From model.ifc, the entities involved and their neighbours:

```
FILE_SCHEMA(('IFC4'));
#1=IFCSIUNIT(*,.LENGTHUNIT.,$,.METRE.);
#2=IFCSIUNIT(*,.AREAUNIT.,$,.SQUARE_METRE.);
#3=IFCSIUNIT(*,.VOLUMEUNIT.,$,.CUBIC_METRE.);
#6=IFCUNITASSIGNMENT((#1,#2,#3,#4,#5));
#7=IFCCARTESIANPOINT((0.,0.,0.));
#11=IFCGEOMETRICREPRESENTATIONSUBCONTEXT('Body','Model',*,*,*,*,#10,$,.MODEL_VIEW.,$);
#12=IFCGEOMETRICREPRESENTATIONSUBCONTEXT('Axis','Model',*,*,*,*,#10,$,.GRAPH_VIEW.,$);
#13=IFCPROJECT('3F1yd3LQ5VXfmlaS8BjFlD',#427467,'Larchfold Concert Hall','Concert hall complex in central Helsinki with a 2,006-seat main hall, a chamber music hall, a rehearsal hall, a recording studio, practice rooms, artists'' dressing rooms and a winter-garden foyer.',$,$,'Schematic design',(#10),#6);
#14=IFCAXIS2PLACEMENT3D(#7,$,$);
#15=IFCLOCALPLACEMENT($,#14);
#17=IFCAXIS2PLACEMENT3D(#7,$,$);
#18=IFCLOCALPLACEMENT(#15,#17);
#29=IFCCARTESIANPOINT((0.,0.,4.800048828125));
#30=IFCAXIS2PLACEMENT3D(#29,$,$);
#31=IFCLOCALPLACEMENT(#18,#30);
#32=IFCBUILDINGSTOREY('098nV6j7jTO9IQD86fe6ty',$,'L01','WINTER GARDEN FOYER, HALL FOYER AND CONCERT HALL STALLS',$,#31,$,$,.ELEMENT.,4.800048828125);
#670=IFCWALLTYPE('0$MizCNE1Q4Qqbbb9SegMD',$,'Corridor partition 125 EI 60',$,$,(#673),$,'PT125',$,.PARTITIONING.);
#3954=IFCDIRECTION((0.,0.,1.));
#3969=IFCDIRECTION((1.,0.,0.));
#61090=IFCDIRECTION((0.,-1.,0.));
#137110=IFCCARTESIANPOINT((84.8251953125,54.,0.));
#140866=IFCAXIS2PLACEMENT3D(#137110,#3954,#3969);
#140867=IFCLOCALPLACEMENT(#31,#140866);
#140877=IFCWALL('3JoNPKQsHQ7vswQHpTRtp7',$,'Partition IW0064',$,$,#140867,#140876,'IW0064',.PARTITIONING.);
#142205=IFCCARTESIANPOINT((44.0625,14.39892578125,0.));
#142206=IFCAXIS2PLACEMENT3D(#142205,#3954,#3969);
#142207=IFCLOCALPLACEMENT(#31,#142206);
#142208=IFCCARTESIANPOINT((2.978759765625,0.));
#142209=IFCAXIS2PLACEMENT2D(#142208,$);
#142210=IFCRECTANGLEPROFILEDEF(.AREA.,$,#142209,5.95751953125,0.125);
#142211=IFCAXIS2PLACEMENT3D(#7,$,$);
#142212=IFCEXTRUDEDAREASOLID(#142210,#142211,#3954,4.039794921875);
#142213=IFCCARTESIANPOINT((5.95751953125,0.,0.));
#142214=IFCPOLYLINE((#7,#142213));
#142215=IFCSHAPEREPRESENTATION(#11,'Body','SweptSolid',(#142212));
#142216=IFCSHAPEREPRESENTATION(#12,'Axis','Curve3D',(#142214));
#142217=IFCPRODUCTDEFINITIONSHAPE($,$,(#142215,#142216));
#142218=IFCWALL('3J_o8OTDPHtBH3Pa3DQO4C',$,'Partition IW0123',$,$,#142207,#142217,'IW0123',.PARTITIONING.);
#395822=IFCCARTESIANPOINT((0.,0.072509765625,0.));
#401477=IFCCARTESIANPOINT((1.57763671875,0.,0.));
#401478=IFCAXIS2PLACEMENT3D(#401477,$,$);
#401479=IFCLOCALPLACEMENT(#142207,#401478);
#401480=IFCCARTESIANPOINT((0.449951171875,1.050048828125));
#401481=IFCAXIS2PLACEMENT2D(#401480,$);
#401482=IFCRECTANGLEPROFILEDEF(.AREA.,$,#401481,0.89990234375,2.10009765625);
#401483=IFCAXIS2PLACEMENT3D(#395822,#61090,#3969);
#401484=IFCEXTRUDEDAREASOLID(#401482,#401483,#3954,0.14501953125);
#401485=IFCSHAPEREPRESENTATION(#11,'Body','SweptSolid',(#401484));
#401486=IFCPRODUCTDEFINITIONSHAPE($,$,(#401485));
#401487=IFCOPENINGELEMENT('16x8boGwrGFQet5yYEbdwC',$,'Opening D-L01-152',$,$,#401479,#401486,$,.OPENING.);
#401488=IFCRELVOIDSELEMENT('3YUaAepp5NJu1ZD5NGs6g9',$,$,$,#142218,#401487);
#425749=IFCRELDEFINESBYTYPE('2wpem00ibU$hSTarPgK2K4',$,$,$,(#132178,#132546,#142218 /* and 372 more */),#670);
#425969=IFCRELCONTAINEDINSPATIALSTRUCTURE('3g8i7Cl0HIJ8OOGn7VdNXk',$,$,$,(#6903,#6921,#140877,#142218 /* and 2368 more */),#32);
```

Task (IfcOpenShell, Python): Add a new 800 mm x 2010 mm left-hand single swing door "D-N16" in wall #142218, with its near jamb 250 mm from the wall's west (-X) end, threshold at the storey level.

```python
import numpy as np
import ifcopenshell
import ifcopenshell.api.feature
import ifcopenshell.api.geometry
import ifcopenshell.api.root
import ifcopenshell.api.spatial
import ifcopenshell.geom
import ifcopenshell.util.element
import ifcopenshell.util.placement
import ifcopenshell.util.representation
import ifcopenshell.util.shape
import ifcopenshell.util.unit

model = ifcopenshell.open("model.ifc")
unit_scale = ifcopenshell.util.unit.calculate_unit_scale(model)
settings = ifcopenshell.geom.settings()


def volume(element):
    """Net volume in cubic metres, openings subtracted."""
    shape = ifcopenshell.geom.create_shape(settings, element)
    return ifcopenshell.util.shape.get_volume(shape.geometry)


wall = model.by_guid("3J_o8OTDPHtBH3Pa3DQO4C")
storey = ifcopenshell.util.element.get_container(wall, ifc_class="IfcBuildingStorey")
context = ifcopenshell.util.representation.get_context(model, "Model", "Body", "MODEL_VIEW")
before = volume(wall)

width, height, from_end, sill = 0.8, 2.01, 0.25, 0.0  # metres

# The wall runs along its own X axis, and the end named is its -X end.
wall_shape = ifcopenshell.geom.create_shape(settings, wall)
x, y, z = ifcopenshell.util.shape.get_vertices(wall_shape.geometry).T
start = x.min() + from_end
face, thickness = float(y.min()), float(y.max() - y.min())
wall_matrix = ifcopenshell.util.placement.get_local_placement(wall.ObjectPlacement)
level = ifcopenshell.util.placement.get_local_placement(storey.ObjectPlacement)[2, 3]


def in_wall(x, y):
    """Placement at x, y metres in the wall's axes, at sill height."""
    matrix = wall_matrix.copy()
    matrix[:, 3] = wall_matrix @ np.array([x / unit_scale, y / unit_scale, 0.0, 1.0])
    matrix[2, 3] = level + sill / unit_scale
    return matrix


# Opening: a box that overshoots both wall faces by 50 mm.
opening = ifcopenshell.api.root.create_entity(model, ifc_class="IfcOpeningElement", predefined_type="OPENING")
box = ifcopenshell.api.geometry.add_wall_representation(
    model, context=context, length=width, height=height, thickness=thickness + 0.1
)
ifcopenshell.api.geometry.assign_representation(model, product=opening, representation=box)
ifcopenshell.api.geometry.edit_object_placement(model, product=opening, matrix=in_wall(start, face - 0.05), is_si=False)
ifcopenshell.api.feature.add_feature(model, feature=opening, element=wall)

door = ifcopenshell.api.root.create_entity(model, ifc_class="IfcDoor", name="D-N16", predefined_type="DOOR")
door.OverallWidth, door.OverallHeight = width / unit_scale, height / unit_scale
door.OperationType = "SINGLE_SWING_LEFT"
body = ifcopenshell.api.geometry.add_door_representation(
    model,
    context=context,
    overall_width=door.OverallWidth,
    overall_height=door.OverallHeight,
    operation_type="SINGLE_SWING_LEFT",
    lining_properties={"LiningDepth": thickness / unit_scale, "ThresholdDepth": thickness / unit_scale},
)
ifcopenshell.api.geometry.assign_representation(model, product=door, representation=body)
ifcopenshell.api.spatial.assign_container(model, products=[door], relating_structure=storey)
ifcopenshell.api.feature.add_filling(model, opening=opening, element=door)

# The lining spans the wall, so the door starts at the wall face.
ifcopenshell.api.geometry.edit_object_placement(model, product=door, matrix=in_wall(start, face), is_si=False)

after = volume(wall)

print(f"wall volume {before:.3f} -> {after:.3f} m3")

model.write("model_v2.ifc")
```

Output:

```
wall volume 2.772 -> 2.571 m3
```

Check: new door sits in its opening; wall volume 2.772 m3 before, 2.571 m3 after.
